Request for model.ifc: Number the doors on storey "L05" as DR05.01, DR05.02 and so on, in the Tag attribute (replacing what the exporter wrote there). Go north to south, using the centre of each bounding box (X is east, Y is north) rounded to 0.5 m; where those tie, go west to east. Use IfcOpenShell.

First a look at what the model holds.

```python
import ifcopenshell
import ifcopenshell.util.element
import ifcopenshell.util.placement

model = ifcopenshell.open("model.ifc")
print(model.schema)
storey = next(s for s in model.by_type("IfcBuildingStorey") if s.Name == "L05")
doors = [e for e in ifcopenshell.util.element.get_decomposition(storey) if e.is_a("IfcDoor")]
for e in sorted(doors, key=lambda e: e.id()):
    origin = ifcopenshell.util.placement.get_local_placement(e.ObjectPlacement)[:3, 3]
    print(e.id(), e.Tag, e.Name, origin.round(2) + 0.0, sep=" | ")
```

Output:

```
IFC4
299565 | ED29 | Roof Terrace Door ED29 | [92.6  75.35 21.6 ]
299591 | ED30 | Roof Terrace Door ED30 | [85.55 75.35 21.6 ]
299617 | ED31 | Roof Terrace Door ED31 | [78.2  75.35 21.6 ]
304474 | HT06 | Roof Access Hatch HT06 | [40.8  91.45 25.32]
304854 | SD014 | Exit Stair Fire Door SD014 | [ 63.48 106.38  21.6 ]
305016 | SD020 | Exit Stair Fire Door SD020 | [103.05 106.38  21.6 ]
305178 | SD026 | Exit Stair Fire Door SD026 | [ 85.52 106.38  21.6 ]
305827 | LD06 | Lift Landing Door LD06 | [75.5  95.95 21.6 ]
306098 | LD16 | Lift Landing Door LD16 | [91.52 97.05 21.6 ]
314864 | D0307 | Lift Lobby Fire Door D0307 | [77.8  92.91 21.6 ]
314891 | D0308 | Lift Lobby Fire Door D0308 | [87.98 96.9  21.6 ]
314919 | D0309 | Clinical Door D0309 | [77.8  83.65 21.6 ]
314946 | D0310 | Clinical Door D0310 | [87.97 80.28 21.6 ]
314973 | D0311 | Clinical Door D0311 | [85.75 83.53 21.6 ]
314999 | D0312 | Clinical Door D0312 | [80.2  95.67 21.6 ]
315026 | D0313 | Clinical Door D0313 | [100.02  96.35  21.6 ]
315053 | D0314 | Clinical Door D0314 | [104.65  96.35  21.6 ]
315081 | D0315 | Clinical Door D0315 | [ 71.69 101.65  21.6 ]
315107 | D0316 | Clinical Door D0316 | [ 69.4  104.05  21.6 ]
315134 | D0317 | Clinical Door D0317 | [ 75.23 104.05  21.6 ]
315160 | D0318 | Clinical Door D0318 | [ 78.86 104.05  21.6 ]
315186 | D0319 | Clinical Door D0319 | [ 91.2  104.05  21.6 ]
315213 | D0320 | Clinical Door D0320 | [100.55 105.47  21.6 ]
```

```python
import ifcopenshell
import ifcopenshell.geom
import ifcopenshell.util.element
import ifcopenshell.util.shape

model = ifcopenshell.open("model.ifc")
settings = ifcopenshell.geom.settings()
settings.set("use-world-coords", True)


def centre(element):
    shape = ifcopenshell.geom.create_shape(settings, element)
    return ifcopenshell.util.shape.get_bbox_centroid(shape.geometry)


storey = next(s for s in model.by_type("IfcBuildingStorey") if s.Name == "L05")
doors = [e for e in ifcopenshell.util.element.get_decomposition(storey) if e.is_a("IfcDoor")]

# Insertion points can sit at a corner or the storey origin, so sort by the geometry (in metres).
centres = {e: centre(e) for e in doors}
doors.sort(key=lambda e: (-round(centres[e][1] / 0.5), centres[e][0]))

for i, e in enumerate(doors, start=1):
    number = f"DR05.{i:02d}"
    e.Tag = number
    print(e.id(), number)

model.write("model-out.ifc")
```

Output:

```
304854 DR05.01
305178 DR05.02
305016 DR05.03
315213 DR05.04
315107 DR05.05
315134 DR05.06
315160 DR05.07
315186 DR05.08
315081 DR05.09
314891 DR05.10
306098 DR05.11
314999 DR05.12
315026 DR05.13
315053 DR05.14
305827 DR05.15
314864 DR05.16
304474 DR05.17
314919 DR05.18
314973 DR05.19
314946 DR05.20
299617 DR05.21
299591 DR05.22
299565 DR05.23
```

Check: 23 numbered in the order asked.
